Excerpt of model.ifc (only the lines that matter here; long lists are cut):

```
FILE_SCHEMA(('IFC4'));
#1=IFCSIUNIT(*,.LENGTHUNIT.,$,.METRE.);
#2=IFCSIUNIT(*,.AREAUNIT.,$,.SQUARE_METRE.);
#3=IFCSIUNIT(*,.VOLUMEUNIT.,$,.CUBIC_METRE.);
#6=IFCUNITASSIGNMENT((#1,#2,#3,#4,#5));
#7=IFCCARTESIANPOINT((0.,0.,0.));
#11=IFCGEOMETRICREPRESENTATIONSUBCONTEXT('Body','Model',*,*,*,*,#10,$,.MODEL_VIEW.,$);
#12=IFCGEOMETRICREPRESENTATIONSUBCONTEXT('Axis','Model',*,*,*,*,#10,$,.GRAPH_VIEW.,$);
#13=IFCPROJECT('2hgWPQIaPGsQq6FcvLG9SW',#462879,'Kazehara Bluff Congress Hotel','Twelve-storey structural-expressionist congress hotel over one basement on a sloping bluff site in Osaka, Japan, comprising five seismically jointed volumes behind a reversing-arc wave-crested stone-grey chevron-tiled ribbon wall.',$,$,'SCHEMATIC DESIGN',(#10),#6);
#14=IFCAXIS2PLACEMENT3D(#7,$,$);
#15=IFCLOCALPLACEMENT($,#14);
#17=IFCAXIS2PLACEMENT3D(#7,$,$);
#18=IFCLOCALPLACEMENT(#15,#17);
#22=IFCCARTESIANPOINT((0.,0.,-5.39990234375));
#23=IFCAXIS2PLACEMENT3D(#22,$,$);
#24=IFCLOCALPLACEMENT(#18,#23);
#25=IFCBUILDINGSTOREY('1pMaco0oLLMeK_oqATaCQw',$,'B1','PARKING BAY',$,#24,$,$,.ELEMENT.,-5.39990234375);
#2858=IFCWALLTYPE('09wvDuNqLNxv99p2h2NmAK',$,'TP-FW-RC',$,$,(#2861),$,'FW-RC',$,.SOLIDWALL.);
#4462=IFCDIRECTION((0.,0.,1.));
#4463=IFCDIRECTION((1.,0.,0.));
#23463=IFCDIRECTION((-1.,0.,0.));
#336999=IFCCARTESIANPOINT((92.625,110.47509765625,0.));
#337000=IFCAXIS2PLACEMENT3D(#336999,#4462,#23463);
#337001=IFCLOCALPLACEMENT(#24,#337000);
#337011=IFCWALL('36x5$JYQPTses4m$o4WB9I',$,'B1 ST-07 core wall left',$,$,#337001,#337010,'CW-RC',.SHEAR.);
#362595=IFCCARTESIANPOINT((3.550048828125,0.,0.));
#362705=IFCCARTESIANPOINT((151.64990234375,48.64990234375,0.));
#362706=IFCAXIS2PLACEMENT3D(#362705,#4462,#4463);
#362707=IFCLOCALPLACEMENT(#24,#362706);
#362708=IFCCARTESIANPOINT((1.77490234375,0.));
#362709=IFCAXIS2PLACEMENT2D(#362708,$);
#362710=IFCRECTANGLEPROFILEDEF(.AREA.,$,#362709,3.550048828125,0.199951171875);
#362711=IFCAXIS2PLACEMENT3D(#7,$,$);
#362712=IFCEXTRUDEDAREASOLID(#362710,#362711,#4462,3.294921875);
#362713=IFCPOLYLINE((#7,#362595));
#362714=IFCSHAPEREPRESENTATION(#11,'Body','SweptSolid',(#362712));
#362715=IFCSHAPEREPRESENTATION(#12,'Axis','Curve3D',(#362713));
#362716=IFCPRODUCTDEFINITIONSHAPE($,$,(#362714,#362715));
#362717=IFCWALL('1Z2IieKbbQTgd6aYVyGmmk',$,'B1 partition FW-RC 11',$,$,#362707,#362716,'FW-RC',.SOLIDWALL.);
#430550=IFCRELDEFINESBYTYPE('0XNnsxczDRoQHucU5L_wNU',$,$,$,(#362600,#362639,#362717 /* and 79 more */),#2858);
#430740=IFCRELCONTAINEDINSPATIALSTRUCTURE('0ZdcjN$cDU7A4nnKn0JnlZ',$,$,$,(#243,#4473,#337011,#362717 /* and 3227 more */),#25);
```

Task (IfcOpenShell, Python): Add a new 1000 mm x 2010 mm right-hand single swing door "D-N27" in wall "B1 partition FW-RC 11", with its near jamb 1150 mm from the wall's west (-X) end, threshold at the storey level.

```python
import numpy as np
import ifcopenshell
import ifcopenshell.api.feature
import ifcopenshell.api.geometry
import ifcopenshell.api.root
import ifcopenshell.api.spatial
import ifcopenshell.geom
import ifcopenshell.util.element
import ifcopenshell.util.placement
import ifcopenshell.util.representation
import ifcopenshell.util.shape
import ifcopenshell.util.unit

model = ifcopenshell.open("model.ifc")
unit_scale = ifcopenshell.util.unit.calculate_unit_scale(model)
settings = ifcopenshell.geom.settings()


def volume(element):
    """Net volume in cubic metres, openings subtracted."""
    shape = ifcopenshell.geom.create_shape(settings, element)
    return ifcopenshell.util.shape.get_volume(shape.geometry)


wall = model.by_guid("1Z2IieKbbQTgd6aYVyGmmk")
storey = ifcopenshell.util.element.get_container(wall, ifc_class="IfcBuildingStorey")
context = ifcopenshell.util.representation.get_context(model, "Model", "Body", "MODEL_VIEW")
before = volume(wall)

width, height, from_end, sill = 1, 2.01, 1.15, 0.0  # metres

# The wall runs along its own X axis, and the end named is its -X end.
wall_shape = ifcopenshell.geom.create_shape(settings, wall)
x, y, z = ifcopenshell.util.shape.get_vertices(wall_shape.geometry).T
start = x.min() + from_end
face, thickness = float(y.min()), float(y.max() - y.min())
wall_matrix = ifcopenshell.util.placement.get_local_placement(wall.ObjectPlacement)
level = ifcopenshell.util.placement.get_local_placement(storey.ObjectPlacement)[2, 3]


def in_wall(x, y):
    """Placement at x, y metres in the wall's axes, at sill height."""
    matrix = wall_matrix.copy()
    matrix[:, 3] = wall_matrix @ np.array([x / unit_scale, y / unit_scale, 0.0, 1.0])
    matrix[2, 3] = level + sill / unit_scale
    return matrix


# Opening: a box that overshoots both wall faces by 50 mm.
opening = ifcopenshell.api.root.create_entity(model, ifc_class="IfcOpeningElement", predefined_type="OPENING")
box = ifcopenshell.api.geometry.add_wall_representation(
    model, context=context, length=width, height=height, thickness=thickness + 0.1
)
ifcopenshell.api.geometry.assign_representation(model, product=opening, representation=box)
ifcopenshell.api.geometry.edit_object_placement(model, product=opening, matrix=in_wall(start, face - 0.05), is_si=False)
ifcopenshell.api.feature.add_feature(model, feature=opening, element=wall)

door = ifcopenshell.api.root.create_entity(model, ifc_class="IfcDoor", name="D-N27", predefined_type="DOOR")
door.OverallWidth, door.OverallHeight = width / unit_scale, height / unit_scale
door.OperationType = "SINGLE_SWING_RIGHT"
body = ifcopenshell.api.geometry.add_door_representation(
    model,
    context=context,
    overall_width=door.OverallWidth,
    overall_height=door.OverallHeight,
    operation_type="SINGLE_SWING_RIGHT",
    lining_properties={"LiningDepth": thickness / unit_scale, "ThresholdDepth": thickness / unit_scale},
)
ifcopenshell.api.geometry.assign_representation(model, product=door, representation=body)
ifcopenshell.api.spatial.assign_container(model, products=[door], relating_structure=storey)
ifcopenshell.api.feature.add_filling(model, opening=opening, element=door)

# The lining spans the wall, so the door starts at the wall face.
ifcopenshell.api.geometry.edit_object_placement(model, product=door, matrix=in_wall(start, face), is_si=False)

after = volume(wall)

print(f"wall volume {before:.3f} -> {after:.3f} m3")

model.write("model_v2.ifc")
```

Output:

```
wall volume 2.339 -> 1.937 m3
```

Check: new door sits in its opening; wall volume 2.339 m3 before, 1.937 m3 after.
